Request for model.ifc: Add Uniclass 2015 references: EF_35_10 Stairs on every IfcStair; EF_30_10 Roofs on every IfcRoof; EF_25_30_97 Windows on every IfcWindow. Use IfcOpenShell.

First a look at what the model holds.

```python
import ifcopenshell

model = ifcopenshell.open("model.ifc")
print(model.schema)
print("classifications:", [c.Name for c in model.by_type("IfcClassification")])
for ifc_class in ("IfcDoor", "IfcRoof", "IfcStair", "IfcWall", "IfcWindow"):
    print(ifc_class, len(model.by_type(ifc_class)))
```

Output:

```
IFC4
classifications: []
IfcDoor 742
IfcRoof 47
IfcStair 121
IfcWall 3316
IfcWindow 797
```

```python
import ifcopenshell
import ifcopenshell.api.classification

model = ifcopenshell.open("model.ifc")

system = ifcopenshell.api.classification.add_classification(model, classification="Uniclass 2015")

codes = {
    "IfcStair": ("EF_35_10", "Stairs"),
    "IfcRoof": ("EF_30_10", "Roofs"),
    "IfcWindow": ("EF_25_30_97", "Windows"),
}
for ifc_class, (code, name) in codes.items():
    products = model.by_type(ifc_class)
    ifcopenshell.api.classification.add_reference(
        model, products=products, classification=system, identification=code, name=name
    )
    print(code, len(products))

model.write("model_rev.ifc")
```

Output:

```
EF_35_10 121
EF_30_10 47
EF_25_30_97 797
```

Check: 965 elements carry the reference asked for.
